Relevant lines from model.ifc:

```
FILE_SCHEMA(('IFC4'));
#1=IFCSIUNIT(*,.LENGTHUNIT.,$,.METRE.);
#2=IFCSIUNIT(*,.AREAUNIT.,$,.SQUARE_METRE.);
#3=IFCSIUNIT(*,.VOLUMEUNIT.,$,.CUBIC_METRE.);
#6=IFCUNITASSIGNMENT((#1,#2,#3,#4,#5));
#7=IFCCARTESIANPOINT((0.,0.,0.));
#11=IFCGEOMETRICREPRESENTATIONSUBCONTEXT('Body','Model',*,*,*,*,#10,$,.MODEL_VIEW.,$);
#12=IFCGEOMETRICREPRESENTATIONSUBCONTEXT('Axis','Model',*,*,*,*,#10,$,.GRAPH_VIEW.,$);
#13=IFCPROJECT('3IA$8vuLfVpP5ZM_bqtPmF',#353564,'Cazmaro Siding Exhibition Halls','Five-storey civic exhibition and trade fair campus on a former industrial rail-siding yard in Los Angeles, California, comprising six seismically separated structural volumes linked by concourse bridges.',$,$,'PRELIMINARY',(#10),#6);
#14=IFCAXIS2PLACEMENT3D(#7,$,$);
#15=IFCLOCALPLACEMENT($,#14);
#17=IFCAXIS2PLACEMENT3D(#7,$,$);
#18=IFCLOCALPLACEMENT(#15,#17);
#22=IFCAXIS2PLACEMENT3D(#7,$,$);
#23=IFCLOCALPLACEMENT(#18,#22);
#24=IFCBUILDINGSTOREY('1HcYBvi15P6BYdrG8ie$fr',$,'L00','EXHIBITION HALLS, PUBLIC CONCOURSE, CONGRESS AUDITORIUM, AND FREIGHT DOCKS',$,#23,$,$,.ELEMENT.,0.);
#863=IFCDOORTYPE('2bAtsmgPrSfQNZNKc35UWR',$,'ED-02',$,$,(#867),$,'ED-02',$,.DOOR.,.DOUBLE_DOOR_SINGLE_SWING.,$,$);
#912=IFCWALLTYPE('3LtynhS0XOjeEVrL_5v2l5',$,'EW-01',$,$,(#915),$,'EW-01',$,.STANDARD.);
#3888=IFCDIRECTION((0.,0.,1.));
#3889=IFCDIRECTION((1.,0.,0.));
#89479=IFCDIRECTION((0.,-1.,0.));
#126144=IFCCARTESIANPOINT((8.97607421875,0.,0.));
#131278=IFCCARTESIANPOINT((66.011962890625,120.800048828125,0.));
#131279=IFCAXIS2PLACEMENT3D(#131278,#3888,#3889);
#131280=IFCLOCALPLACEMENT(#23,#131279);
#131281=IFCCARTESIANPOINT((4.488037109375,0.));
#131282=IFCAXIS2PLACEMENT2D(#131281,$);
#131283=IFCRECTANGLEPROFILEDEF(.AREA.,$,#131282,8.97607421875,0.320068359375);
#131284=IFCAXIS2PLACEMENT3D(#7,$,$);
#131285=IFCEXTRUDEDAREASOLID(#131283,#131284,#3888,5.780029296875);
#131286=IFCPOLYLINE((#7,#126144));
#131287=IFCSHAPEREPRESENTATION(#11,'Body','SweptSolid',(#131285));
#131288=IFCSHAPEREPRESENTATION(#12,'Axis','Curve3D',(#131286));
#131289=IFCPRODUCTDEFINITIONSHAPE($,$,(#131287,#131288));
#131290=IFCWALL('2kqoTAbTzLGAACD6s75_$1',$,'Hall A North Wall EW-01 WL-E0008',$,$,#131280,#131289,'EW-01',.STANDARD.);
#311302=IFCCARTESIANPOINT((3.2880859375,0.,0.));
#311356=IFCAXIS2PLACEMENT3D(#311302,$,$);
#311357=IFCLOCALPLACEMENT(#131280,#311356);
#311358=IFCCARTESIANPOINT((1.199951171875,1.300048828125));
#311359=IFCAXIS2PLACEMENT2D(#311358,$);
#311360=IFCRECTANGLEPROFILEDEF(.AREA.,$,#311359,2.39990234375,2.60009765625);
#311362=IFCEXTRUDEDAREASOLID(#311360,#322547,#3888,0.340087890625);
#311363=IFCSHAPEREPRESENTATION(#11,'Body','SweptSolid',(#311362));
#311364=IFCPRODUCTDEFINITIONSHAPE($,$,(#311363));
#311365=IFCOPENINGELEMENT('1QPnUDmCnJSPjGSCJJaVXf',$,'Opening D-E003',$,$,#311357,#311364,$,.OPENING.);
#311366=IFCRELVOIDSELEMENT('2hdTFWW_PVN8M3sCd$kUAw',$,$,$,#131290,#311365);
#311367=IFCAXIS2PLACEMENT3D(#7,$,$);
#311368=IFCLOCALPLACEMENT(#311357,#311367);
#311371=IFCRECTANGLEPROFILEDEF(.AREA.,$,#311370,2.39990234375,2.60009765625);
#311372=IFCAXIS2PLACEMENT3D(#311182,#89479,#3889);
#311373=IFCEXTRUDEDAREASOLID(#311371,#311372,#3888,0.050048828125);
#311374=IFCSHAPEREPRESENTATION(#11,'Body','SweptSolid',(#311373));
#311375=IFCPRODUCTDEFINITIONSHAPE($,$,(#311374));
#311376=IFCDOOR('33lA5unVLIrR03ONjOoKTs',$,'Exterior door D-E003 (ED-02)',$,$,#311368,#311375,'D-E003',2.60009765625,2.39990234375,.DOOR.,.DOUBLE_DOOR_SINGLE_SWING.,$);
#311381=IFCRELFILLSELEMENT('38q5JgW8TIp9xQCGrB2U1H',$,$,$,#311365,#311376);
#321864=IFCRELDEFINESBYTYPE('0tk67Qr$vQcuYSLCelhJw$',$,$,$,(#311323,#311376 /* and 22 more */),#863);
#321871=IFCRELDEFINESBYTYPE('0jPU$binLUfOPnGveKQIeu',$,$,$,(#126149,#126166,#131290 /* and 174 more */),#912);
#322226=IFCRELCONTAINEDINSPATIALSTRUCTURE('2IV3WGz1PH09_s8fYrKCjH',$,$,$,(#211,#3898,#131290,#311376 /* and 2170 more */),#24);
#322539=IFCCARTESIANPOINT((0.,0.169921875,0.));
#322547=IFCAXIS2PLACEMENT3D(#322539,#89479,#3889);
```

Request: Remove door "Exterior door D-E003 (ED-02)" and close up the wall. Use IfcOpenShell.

```python
import ifcopenshell
import ifcopenshell.api.feature
import ifcopenshell.api.root
import ifcopenshell.geom
import ifcopenshell.util.shape

model = ifcopenshell.open("model.ifc")
settings = ifcopenshell.geom.settings()


def volume(element):
    """Net volume in cubic metres, openings subtracted."""
    shape = ifcopenshell.geom.create_shape(settings, element)
    return ifcopenshell.util.shape.get_volume(shape.geometry)


door = model.by_id(311376)
opening = door.FillsVoids[0].RelatingOpeningElement
wall = opening.VoidsElements[0].RelatingBuildingElement
before = volume(wall)

ifcopenshell.api.root.remove_product(model, product=door)
ifcopenshell.api.feature.remove_feature(model, feature=opening)

after = volume(wall)

print(f"wall volume {before:.3f} -> {after:.3f} m3")

model.write("model-out.ifc")
```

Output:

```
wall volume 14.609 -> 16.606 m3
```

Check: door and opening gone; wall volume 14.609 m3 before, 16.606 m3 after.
